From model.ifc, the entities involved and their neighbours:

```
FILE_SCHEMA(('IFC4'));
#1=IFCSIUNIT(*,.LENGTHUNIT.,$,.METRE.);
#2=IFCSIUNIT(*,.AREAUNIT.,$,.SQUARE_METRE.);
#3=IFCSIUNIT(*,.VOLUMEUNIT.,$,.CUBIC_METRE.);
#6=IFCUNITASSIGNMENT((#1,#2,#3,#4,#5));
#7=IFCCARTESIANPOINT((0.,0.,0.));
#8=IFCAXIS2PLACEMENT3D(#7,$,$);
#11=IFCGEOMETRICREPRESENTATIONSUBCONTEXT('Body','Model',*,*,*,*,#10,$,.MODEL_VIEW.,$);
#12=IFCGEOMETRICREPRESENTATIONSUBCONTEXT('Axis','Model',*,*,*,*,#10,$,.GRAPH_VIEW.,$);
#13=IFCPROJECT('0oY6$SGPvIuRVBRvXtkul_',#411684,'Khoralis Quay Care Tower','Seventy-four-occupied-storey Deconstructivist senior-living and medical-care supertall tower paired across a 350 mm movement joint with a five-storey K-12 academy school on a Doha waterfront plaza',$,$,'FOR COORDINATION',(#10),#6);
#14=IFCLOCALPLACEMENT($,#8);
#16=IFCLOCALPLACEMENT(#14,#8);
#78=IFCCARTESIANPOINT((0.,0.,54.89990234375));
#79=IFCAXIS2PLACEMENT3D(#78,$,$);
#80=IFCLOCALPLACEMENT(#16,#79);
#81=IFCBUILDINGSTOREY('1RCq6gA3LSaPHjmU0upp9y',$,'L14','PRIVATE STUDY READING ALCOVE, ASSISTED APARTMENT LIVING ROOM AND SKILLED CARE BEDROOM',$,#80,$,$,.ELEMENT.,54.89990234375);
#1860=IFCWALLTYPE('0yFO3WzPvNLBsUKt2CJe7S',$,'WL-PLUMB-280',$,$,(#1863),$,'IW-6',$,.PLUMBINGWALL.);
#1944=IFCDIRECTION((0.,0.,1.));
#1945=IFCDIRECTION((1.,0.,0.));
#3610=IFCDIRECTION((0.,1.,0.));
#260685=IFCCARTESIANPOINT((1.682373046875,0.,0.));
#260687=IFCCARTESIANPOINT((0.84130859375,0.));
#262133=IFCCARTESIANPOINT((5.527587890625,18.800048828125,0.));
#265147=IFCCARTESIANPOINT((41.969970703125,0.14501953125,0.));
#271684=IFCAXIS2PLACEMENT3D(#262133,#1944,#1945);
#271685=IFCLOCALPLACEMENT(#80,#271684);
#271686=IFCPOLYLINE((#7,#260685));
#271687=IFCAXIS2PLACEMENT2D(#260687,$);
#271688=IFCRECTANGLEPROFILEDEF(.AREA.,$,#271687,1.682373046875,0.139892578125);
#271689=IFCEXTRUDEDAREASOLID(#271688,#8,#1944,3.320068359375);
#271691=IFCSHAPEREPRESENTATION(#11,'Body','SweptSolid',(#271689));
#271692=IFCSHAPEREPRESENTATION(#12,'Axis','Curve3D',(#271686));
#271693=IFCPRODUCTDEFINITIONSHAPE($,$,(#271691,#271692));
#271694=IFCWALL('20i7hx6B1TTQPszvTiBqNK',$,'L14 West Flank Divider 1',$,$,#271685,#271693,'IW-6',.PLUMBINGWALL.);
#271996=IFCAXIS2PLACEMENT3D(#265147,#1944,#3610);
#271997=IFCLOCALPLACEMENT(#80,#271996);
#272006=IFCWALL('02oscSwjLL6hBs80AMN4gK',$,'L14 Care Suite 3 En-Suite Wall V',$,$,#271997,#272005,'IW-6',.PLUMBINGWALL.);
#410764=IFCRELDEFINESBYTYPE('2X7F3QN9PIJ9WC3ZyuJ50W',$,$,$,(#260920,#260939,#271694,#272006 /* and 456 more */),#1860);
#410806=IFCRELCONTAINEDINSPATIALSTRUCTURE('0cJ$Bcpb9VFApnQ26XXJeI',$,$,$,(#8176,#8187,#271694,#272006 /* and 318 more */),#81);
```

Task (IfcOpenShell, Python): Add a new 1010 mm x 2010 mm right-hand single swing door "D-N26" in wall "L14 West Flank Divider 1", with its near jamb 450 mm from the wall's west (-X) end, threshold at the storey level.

```python
import numpy as np
import ifcopenshell
import ifcopenshell.api.feature
import ifcopenshell.api.geometry
import ifcopenshell.api.root
import ifcopenshell.api.spatial
import ifcopenshell.geom
import ifcopenshell.util.element
import ifcopenshell.util.placement
import ifcopenshell.util.representation
import ifcopenshell.util.shape
import ifcopenshell.util.unit

model = ifcopenshell.open("model.ifc")
unit_scale = ifcopenshell.util.unit.calculate_unit_scale(model)
settings = ifcopenshell.geom.settings()


def volume(element):
    """Net volume in cubic metres, openings subtracted."""
    shape = ifcopenshell.geom.create_shape(settings, element)
    return ifcopenshell.util.shape.get_volume(shape.geometry)


wall = model.by_guid("20i7hx6B1TTQPszvTiBqNK")
storey = ifcopenshell.util.element.get_container(wall, ifc_class="IfcBuildingStorey")
context = ifcopenshell.util.representation.get_context(model, "Model", "Body", "MODEL_VIEW")
before = volume(wall)

width, height, from_end, sill = 1.01, 2.01, 0.45, 0.0  # metres

# The wall runs along its own X axis, and the end named is its -X end.
wall_shape = ifcopenshell.geom.create_shape(settings, wall)
x, y, z = ifcopenshell.util.shape.get_vertices(wall_shape.geometry).T
start = x.min() + from_end
face, thickness = float(y.min()), float(y.max() - y.min())
wall_matrix = ifcopenshell.util.placement.get_local_placement(wall.ObjectPlacement)
level = ifcopenshell.util.placement.get_local_placement(storey.ObjectPlacement)[2, 3]


def in_wall(x, y):
    """Placement at x, y metres in the wall's axes, at sill height."""
    matrix = wall_matrix.copy()
    matrix[:, 3] = wall_matrix @ np.array([x / unit_scale, y / unit_scale, 0.0, 1.0])
    matrix[2, 3] = level + sill / unit_scale
    return matrix


# Opening: a box that overshoots both wall faces by 50 mm.
opening = ifcopenshell.api.root.create_entity(model, ifc_class="IfcOpeningElement", predefined_type="OPENING")
box = ifcopenshell.api.geometry.add_wall_representation(
    model, context=context, length=width, height=height, thickness=thickness + 0.1
)
ifcopenshell.api.geometry.assign_representation(model, product=opening, representation=box)
ifcopenshell.api.geometry.edit_object_placement(model, product=opening, matrix=in_wall(start, face - 0.05), is_si=False)
ifcopenshell.api.feature.add_feature(model, feature=opening, element=wall)

door = ifcopenshell.api.root.create_entity(model, ifc_class="IfcDoor", name="D-N26", predefined_type="DOOR")
door.OverallWidth, door.OverallHeight = width / unit_scale, height / unit_scale
door.OperationType = "SINGLE_SWING_RIGHT"
body = ifcopenshell.api.geometry.add_door_representation(
    model,
    context=context,
    overall_width=door.OverallWidth,
    overall_height=door.OverallHeight,
    operation_type="SINGLE_SWING_RIGHT",
    lining_properties={"LiningDepth": thickness / unit_scale, "ThresholdDepth": thickness / unit_scale},
)
ifcopenshell.api.geometry.assign_representation(model, product=door, representation=body)
ifcopenshell.api.spatial.assign_container(model, products=[door], relating_structure=storey)
ifcopenshell.api.feature.add_filling(model, opening=opening, element=door)

# The lining spans the wall, so the door starts at the wall face.
ifcopenshell.api.geometry.edit_object_placement(model, product=door, matrix=in_wall(start, face), is_si=False)

after = volume(wall)

print(f"wall volume {before:.3f} -> {after:.3f} m3")

model.write("model_updated.ifc")
```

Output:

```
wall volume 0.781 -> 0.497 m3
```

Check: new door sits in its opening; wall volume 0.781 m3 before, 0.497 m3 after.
